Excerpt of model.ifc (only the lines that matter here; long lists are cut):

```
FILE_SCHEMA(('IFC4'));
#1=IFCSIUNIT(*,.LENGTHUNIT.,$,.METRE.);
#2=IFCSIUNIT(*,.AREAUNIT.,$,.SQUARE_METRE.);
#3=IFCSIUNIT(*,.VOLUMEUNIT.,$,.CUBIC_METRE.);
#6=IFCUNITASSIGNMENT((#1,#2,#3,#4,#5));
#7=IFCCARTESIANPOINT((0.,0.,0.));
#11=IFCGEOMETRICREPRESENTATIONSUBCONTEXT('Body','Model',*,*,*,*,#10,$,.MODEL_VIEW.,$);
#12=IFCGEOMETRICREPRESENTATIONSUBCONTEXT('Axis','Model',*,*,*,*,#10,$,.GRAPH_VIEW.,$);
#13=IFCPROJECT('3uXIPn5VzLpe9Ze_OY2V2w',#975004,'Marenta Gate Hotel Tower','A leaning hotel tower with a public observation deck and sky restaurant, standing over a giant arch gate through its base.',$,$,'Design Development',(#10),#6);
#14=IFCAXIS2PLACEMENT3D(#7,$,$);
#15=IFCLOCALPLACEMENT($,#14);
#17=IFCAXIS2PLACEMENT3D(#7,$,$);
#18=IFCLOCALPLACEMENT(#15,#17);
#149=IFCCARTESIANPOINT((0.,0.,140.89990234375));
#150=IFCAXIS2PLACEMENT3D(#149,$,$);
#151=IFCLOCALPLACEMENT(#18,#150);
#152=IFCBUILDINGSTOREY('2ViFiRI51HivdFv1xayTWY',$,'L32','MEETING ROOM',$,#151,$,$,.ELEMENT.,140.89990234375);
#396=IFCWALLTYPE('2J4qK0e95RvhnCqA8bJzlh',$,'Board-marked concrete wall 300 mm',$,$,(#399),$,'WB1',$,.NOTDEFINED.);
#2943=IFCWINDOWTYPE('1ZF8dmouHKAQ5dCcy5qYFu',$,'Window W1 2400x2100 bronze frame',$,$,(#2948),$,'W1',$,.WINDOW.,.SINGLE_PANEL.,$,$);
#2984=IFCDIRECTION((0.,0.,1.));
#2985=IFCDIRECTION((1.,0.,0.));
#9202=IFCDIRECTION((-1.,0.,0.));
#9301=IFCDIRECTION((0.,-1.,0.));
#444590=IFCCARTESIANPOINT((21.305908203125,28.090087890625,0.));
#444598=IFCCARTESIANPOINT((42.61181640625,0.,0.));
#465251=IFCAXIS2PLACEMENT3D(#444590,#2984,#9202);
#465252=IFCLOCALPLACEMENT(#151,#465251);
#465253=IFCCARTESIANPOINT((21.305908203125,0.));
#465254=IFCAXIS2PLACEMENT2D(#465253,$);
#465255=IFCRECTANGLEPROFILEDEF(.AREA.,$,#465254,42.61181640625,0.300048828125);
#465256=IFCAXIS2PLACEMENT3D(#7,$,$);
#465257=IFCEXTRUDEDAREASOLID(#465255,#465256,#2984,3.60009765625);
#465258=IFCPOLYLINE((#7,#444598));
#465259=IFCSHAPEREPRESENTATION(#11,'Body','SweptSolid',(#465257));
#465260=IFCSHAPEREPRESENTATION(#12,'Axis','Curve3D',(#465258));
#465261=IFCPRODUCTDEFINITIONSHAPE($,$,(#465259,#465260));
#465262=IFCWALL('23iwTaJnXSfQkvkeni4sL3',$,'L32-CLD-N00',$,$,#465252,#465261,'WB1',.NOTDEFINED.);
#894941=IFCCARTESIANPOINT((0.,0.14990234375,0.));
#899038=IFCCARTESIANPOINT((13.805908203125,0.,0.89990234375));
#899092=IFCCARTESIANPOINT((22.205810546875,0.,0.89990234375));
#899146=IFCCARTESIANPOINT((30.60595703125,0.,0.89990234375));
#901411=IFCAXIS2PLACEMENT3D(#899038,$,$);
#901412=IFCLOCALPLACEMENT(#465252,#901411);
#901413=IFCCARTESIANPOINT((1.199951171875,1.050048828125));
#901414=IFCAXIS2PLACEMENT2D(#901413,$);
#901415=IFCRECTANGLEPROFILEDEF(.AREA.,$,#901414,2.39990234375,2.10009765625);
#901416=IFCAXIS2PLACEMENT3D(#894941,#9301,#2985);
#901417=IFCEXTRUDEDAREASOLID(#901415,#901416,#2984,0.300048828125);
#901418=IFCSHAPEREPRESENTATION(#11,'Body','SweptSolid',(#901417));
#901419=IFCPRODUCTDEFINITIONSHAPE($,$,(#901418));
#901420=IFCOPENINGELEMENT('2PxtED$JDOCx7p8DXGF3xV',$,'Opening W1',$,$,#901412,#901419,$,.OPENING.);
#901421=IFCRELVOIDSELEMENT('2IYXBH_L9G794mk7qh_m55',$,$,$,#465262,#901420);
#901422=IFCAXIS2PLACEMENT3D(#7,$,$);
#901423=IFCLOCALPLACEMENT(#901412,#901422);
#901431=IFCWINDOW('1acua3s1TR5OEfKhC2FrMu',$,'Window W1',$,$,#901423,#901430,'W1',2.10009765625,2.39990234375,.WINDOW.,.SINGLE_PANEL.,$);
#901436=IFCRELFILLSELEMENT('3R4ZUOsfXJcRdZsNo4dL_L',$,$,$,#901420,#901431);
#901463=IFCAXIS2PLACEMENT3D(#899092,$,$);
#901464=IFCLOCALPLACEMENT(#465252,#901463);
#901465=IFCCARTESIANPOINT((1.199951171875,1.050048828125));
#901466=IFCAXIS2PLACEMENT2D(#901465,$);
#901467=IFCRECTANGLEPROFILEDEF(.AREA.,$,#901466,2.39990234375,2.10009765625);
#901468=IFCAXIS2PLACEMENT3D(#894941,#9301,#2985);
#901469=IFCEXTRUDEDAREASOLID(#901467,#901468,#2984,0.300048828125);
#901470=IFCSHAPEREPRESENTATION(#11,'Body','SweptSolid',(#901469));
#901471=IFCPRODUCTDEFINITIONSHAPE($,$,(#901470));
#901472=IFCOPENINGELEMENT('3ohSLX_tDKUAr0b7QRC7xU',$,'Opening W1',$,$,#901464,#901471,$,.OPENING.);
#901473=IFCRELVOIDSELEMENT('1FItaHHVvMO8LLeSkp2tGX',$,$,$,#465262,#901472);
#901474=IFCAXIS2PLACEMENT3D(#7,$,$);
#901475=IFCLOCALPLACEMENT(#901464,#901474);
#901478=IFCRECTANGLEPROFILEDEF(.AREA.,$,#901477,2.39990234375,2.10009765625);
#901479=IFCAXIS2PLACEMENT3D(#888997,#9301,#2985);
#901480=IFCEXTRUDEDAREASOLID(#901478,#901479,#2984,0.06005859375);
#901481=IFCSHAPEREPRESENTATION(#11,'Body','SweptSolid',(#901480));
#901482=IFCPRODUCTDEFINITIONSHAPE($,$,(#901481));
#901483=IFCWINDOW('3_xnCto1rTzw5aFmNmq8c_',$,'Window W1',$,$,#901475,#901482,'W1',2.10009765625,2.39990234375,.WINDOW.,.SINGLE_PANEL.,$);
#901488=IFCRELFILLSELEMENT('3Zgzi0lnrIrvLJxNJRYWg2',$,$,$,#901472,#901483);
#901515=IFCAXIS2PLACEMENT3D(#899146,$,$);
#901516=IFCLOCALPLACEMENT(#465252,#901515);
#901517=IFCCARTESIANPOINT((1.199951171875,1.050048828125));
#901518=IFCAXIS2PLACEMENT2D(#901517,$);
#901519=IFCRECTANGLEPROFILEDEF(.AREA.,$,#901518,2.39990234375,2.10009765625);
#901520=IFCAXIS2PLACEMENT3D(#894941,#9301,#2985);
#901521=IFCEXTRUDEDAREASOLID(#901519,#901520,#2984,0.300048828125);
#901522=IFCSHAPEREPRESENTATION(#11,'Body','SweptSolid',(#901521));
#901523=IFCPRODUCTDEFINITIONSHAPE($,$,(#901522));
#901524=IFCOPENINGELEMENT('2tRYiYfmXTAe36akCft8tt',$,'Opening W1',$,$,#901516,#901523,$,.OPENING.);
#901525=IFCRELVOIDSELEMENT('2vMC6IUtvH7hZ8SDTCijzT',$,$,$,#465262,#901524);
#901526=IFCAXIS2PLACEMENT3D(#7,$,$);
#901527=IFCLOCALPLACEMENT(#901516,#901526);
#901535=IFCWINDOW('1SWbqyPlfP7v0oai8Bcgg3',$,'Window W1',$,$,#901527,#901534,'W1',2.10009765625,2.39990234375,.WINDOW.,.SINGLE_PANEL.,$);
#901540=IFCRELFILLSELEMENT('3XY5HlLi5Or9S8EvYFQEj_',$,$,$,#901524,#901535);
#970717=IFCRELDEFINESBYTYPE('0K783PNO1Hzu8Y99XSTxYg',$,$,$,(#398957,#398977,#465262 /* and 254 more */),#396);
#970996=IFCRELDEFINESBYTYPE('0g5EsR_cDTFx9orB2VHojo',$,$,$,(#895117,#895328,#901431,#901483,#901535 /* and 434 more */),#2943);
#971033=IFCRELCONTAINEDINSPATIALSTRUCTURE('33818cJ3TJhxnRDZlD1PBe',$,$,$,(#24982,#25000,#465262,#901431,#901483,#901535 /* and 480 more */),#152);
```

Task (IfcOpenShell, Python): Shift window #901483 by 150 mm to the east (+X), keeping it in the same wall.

```python
import ifcopenshell
import ifcopenshell.api.geometry
import ifcopenshell.util.placement
import ifcopenshell.util.unit

model = ifcopenshell.open("model.ifc")
unit_scale = ifcopenshell.util.unit.calculate_unit_scale(model)

window = model.by_guid("3_xnCto1rTzw5aFmNmq8c_")
opening = window.FillsVoids[0].RelatingOpeningElement
wall = opening.VoidsElements[0].RelatingBuildingElement

wall_matrix = ifcopenshell.util.placement.get_local_placement(wall.ObjectPlacement)
shift = wall_matrix[:3, 0] * -0.15 / unit_scale
before = ifcopenshell.util.placement.get_local_placement(window.ObjectPlacement)[:3, 3].copy()

# The window is placed relative to its opening, so it follows when the opening moves.
matrix = ifcopenshell.util.placement.get_local_placement(opening.ObjectPlacement)
matrix[:3, 3] += shift
ifcopenshell.api.geometry.edit_object_placement(
    model, product=opening, matrix=matrix, is_si=False, should_transform_children=True
)

after = ifcopenshell.util.placement.get_local_placement(window.ObjectPlacement)[:3, 3]
print("window moved by", (after - before).round(3) + 0.0)

model.write("model-out.ifc")
```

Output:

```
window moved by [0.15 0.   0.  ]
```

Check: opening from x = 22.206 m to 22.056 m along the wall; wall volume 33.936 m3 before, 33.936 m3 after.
